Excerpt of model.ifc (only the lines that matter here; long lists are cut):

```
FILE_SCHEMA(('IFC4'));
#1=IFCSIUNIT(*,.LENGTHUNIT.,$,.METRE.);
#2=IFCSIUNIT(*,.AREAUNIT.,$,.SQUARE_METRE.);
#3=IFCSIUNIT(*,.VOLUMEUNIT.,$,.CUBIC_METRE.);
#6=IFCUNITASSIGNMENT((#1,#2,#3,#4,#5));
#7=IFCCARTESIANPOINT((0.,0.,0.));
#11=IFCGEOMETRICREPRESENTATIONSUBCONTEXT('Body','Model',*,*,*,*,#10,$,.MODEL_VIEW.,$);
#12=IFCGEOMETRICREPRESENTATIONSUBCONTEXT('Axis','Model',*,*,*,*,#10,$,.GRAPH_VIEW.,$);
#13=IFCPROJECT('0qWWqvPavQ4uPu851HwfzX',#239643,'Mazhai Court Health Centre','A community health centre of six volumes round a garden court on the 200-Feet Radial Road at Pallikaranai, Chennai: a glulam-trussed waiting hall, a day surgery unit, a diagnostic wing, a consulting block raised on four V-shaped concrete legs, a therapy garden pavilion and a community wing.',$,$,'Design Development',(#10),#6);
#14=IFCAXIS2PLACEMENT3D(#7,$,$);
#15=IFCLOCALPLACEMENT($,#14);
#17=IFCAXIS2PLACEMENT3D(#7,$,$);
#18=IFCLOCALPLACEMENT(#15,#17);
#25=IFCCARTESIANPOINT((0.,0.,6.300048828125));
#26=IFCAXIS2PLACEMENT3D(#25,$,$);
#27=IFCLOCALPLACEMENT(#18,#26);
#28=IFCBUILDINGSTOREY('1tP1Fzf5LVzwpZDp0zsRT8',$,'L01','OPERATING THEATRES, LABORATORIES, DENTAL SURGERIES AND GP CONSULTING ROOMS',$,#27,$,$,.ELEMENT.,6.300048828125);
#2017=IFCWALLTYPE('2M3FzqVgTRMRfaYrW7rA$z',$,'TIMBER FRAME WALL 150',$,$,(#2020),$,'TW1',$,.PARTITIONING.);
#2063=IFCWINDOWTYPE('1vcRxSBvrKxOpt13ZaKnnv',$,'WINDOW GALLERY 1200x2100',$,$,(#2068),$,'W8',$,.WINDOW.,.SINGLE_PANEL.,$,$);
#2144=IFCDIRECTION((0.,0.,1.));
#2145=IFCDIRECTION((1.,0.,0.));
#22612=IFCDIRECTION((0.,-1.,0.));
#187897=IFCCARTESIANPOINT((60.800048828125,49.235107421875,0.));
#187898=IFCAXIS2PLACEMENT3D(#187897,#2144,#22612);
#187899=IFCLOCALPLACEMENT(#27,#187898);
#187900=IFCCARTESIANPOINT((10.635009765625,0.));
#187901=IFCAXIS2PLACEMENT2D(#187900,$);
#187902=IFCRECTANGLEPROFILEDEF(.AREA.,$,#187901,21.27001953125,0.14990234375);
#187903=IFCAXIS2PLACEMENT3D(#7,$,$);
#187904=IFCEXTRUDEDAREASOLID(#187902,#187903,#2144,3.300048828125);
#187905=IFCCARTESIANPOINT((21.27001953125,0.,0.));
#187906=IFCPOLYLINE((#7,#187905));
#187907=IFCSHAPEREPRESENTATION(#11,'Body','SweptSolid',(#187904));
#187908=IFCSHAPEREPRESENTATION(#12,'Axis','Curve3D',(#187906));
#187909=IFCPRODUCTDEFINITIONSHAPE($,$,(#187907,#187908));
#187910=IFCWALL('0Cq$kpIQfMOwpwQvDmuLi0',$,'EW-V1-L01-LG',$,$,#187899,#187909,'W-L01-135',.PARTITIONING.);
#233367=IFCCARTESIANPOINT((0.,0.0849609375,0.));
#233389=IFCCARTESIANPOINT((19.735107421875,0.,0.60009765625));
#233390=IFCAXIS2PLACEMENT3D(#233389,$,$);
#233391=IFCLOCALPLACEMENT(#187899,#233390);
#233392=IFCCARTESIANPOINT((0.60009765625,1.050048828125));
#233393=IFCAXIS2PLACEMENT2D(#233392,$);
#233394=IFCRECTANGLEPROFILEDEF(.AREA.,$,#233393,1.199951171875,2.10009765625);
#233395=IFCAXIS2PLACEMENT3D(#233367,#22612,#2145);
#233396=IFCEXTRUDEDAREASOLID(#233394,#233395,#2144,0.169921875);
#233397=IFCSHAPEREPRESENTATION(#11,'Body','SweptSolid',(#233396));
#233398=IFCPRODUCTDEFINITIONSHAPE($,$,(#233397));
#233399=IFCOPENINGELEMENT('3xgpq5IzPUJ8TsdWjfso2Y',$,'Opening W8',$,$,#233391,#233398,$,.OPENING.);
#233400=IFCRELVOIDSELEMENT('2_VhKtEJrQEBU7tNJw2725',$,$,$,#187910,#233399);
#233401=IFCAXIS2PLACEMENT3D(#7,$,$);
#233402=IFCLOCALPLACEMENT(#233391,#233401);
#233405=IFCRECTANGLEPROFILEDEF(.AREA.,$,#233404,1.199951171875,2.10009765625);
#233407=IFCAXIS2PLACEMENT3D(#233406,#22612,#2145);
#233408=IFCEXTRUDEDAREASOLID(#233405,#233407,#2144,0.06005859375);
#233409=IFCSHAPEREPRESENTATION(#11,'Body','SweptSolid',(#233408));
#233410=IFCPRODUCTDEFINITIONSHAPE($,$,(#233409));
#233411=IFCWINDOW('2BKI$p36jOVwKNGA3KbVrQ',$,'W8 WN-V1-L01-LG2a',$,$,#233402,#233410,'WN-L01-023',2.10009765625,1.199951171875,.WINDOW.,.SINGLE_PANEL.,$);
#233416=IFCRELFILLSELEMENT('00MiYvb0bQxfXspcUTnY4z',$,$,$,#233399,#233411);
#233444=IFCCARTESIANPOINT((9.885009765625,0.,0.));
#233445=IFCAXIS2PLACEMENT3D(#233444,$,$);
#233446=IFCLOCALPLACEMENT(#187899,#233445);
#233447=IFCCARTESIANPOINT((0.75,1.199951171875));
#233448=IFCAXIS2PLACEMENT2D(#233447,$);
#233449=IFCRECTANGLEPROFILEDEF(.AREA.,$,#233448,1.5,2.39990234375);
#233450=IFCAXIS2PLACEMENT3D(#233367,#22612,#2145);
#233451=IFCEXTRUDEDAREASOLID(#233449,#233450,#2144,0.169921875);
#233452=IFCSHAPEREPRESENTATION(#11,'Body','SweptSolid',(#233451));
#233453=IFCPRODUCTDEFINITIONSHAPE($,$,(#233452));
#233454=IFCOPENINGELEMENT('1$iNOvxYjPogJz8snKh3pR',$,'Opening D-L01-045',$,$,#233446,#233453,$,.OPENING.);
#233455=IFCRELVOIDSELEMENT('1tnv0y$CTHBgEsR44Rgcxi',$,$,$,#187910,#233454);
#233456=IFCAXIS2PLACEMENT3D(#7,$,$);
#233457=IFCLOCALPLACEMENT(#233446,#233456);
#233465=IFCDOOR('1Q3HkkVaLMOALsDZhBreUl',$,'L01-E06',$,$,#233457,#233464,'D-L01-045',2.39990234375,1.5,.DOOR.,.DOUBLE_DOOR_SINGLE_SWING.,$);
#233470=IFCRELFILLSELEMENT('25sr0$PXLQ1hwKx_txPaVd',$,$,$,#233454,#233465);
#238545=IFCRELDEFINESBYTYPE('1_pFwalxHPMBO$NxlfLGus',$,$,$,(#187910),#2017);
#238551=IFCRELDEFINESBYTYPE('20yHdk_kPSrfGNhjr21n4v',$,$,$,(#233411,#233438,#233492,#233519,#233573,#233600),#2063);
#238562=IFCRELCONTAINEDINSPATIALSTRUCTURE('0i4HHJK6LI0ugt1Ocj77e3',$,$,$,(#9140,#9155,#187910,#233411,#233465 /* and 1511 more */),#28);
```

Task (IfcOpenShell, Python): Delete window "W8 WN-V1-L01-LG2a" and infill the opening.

```python
import ifcopenshell
import ifcopenshell.api.feature
import ifcopenshell.api.root
import ifcopenshell.geom
import ifcopenshell.util.shape

model = ifcopenshell.open("model.ifc")
settings = ifcopenshell.geom.settings()


def volume(element):
    """Net volume in cubic metres, openings subtracted."""
    shape = ifcopenshell.geom.create_shape(settings, element)
    return ifcopenshell.util.shape.get_volume(shape.geometry)


window = model.by_guid("2BKI$p36jOVwKNGA3KbVrQ")
opening = window.FillsVoids[0].RelatingOpeningElement
wall = opening.VoidsElements[0].RelatingBuildingElement
before = volume(wall)

ifcopenshell.api.root.remove_product(model, product=window)
ifcopenshell.api.feature.remove_feature(model, feature=opening)

after = volume(wall)

print(f"wall volume {before:.3f} -> {after:.3f} m3")

model.write("model_edited.ifc")
```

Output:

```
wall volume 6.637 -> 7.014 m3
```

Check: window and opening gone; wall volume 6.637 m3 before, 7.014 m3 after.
